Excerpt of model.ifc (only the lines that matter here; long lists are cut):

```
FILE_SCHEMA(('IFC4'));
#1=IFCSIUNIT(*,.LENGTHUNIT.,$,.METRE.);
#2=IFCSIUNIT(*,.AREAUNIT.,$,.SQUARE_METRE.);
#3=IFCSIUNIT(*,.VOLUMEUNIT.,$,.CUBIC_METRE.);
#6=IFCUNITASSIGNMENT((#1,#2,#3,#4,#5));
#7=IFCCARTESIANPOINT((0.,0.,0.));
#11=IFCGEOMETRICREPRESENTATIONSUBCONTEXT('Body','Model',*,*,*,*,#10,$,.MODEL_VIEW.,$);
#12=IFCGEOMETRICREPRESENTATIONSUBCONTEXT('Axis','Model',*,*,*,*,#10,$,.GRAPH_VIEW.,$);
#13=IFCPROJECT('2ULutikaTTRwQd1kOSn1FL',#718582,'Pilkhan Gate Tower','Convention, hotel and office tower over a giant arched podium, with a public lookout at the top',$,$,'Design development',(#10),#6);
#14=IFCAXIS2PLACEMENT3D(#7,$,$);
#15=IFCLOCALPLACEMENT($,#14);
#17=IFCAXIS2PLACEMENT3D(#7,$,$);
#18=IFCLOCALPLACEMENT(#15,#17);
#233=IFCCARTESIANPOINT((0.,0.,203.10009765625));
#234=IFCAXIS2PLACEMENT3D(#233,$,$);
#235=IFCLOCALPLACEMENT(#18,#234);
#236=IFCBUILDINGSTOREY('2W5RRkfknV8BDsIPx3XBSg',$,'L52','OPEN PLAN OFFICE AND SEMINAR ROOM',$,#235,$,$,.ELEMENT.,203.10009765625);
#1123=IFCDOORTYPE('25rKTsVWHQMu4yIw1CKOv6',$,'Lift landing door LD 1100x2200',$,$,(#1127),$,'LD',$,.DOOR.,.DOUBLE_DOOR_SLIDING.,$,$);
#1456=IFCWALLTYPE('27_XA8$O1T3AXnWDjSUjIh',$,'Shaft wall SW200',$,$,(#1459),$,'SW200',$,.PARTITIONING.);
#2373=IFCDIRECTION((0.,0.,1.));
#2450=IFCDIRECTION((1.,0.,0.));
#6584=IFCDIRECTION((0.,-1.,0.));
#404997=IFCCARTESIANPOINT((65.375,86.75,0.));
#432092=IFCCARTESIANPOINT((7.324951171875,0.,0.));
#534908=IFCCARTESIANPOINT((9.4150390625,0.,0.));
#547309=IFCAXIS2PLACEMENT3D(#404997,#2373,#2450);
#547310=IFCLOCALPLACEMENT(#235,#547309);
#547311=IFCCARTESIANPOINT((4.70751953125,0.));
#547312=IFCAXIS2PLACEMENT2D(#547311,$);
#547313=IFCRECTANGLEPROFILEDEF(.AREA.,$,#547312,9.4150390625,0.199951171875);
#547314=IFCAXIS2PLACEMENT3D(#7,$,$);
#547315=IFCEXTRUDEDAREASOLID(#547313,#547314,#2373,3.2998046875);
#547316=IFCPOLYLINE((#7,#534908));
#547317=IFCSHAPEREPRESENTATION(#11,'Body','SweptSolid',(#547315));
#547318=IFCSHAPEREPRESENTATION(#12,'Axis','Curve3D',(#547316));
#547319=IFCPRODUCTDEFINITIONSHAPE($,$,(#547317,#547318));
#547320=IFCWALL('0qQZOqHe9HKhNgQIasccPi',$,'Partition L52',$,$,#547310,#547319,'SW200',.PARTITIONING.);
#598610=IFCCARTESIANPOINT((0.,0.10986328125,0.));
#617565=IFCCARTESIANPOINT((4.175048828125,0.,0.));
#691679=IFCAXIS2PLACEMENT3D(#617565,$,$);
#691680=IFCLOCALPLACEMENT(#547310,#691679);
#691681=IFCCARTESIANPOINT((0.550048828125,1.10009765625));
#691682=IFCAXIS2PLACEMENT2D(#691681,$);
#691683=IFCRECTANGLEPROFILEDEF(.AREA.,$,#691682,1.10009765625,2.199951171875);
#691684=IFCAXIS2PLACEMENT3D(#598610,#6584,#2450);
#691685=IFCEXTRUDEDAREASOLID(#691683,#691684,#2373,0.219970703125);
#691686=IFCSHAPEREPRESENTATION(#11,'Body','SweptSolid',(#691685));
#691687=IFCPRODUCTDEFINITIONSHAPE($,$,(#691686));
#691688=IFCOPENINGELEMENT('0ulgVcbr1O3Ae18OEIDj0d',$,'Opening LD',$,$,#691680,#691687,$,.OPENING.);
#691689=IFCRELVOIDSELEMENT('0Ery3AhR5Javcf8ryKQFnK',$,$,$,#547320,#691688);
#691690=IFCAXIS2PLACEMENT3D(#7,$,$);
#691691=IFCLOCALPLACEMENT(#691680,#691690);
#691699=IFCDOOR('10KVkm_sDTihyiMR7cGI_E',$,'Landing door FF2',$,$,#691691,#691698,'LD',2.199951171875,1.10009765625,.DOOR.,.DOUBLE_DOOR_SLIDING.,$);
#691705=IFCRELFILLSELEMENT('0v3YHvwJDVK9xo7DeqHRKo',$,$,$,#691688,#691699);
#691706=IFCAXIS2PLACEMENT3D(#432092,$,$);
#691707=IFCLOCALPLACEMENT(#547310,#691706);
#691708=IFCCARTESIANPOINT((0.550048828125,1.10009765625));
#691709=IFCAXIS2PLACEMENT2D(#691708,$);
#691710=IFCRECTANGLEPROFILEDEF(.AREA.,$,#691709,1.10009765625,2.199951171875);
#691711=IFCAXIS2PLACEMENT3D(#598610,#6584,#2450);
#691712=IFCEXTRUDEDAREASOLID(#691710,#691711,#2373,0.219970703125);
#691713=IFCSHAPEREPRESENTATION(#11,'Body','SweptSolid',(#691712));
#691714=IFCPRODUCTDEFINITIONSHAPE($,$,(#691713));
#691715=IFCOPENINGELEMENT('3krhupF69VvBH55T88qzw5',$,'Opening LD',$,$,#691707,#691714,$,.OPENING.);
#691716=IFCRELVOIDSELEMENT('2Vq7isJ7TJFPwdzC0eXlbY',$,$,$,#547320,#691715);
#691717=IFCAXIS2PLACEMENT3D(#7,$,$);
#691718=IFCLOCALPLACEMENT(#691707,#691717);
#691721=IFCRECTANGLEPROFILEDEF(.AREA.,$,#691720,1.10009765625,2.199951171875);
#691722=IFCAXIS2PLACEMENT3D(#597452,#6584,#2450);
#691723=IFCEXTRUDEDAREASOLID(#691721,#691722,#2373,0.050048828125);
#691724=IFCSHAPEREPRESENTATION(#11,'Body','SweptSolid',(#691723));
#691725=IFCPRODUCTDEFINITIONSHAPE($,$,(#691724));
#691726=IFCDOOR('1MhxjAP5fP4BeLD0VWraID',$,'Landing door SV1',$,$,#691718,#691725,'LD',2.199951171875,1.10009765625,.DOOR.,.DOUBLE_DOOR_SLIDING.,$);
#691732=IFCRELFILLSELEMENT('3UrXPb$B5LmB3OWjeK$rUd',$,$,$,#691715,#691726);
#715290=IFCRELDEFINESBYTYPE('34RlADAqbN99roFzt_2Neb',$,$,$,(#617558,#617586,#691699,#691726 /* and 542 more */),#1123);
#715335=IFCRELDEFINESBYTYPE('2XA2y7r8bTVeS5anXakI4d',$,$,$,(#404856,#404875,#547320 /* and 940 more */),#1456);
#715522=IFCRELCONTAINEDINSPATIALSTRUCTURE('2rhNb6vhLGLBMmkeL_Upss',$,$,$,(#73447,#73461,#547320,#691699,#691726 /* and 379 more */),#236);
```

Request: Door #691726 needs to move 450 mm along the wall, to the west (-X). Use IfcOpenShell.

```python
import ifcopenshell
import ifcopenshell.api.geometry
import ifcopenshell.util.placement

model = ifcopenshell.open("model.ifc")

door = model.by_guid("1MhxjAP5fP4BeLD0VWraID")
opening = door.FillsVoids[0].RelatingOpeningElement
wall = opening.VoidsElements[0].RelatingBuildingElement

wall_matrix = ifcopenshell.util.placement.get_local_placement(wall.ObjectPlacement)
shift = wall_matrix[:3, 0] * -0.45
before = ifcopenshell.util.placement.get_local_placement(door.ObjectPlacement)[:3, 3].copy()

# The door is placed relative to its opening, so it follows when the opening moves.
matrix = ifcopenshell.util.placement.get_local_placement(opening.ObjectPlacement)
matrix[:3, 3] += shift
ifcopenshell.api.geometry.edit_object_placement(
    model, product=opening, matrix=matrix, is_si=False, should_transform_children=True
)

after = ifcopenshell.util.placement.get_local_placement(door.ObjectPlacement)[:3, 3]
print("door moved by", (after - before).round(3) + 0.0)

model.write("model_rev.ifc")
```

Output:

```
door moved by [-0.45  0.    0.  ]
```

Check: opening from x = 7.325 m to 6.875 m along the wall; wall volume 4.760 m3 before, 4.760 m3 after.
